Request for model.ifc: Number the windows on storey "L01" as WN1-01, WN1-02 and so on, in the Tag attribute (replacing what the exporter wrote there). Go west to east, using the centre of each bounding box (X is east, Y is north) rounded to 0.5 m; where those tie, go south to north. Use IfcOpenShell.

First a look at what the model holds.

```python
import ifcopenshell
import ifcopenshell.util.element
import ifcopenshell.util.placement

model = ifcopenshell.open("model.ifc")
print(model.schema)
storey = next(s for s in model.by_type("IfcBuildingStorey") if s.Name == "L01")
windows = [e for e in ifcopenshell.util.element.get_decomposition(storey) if e.is_a("IfcWindow")]
for e in sorted(windows, key=lambda e: e.id()):
    origin = ifcopenshell.util.placement.get_local_placement(e.ObjectPlacement)[:3, 3]
    print(e.id(), e.Tag, e.Name, origin.round(2) + 0.0, sep=" | ")
```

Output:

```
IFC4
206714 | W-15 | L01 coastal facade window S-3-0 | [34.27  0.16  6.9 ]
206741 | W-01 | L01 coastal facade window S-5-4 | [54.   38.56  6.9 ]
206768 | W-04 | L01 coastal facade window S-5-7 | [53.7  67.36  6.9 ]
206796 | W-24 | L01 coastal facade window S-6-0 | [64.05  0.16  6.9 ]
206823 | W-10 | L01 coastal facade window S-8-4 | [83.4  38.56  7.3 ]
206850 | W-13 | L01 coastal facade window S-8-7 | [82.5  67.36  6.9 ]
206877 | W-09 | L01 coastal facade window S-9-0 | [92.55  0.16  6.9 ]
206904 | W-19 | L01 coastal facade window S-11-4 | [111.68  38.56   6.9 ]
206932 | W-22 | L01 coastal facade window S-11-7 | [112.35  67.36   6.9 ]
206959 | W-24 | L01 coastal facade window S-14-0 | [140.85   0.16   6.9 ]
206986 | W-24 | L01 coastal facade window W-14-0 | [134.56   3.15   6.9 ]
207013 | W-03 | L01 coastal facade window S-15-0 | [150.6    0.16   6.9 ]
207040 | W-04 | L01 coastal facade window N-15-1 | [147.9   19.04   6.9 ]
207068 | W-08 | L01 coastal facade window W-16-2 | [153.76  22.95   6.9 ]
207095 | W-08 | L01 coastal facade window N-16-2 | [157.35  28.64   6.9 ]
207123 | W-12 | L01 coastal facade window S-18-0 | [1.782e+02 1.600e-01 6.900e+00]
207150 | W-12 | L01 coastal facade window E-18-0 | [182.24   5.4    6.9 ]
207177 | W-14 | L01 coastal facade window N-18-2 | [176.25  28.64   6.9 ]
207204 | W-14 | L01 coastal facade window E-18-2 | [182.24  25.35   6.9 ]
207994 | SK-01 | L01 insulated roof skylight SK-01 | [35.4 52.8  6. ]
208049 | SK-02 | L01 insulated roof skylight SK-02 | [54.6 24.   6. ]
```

```python
import ifcopenshell
import ifcopenshell.geom
import ifcopenshell.util.element
import ifcopenshell.util.shape

model = ifcopenshell.open("model.ifc")
settings = ifcopenshell.geom.settings()
settings.set("use-world-coords", True)


def centre(element):
    shape = ifcopenshell.geom.create_shape(settings, element)
    return ifcopenshell.util.shape.get_bbox_centroid(shape.geometry)


storey = next(s for s in model.by_type("IfcBuildingStorey") if s.Name == "L01")
windows = [e for e in ifcopenshell.util.element.get_decomposition(storey) if e.is_a("IfcWindow")]

# Insertion points can sit at a corner or the storey origin, so sort by the geometry (in metres).
centres = {e: centre(e) for e in windows}
windows.sort(key=lambda e: (round(centres[e][0] / 0.5), centres[e][1]))

for i, e in enumerate(windows, start=1):
    number = f"WN1-{i:02d}"
    e.Tag = number
    print(e.id(), number)

model.write("model-out.ifc")
```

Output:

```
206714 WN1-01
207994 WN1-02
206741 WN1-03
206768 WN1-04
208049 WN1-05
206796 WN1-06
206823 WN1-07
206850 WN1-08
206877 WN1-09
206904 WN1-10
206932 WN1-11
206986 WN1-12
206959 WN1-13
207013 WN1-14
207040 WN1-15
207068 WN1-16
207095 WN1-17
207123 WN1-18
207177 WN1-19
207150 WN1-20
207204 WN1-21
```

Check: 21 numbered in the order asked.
